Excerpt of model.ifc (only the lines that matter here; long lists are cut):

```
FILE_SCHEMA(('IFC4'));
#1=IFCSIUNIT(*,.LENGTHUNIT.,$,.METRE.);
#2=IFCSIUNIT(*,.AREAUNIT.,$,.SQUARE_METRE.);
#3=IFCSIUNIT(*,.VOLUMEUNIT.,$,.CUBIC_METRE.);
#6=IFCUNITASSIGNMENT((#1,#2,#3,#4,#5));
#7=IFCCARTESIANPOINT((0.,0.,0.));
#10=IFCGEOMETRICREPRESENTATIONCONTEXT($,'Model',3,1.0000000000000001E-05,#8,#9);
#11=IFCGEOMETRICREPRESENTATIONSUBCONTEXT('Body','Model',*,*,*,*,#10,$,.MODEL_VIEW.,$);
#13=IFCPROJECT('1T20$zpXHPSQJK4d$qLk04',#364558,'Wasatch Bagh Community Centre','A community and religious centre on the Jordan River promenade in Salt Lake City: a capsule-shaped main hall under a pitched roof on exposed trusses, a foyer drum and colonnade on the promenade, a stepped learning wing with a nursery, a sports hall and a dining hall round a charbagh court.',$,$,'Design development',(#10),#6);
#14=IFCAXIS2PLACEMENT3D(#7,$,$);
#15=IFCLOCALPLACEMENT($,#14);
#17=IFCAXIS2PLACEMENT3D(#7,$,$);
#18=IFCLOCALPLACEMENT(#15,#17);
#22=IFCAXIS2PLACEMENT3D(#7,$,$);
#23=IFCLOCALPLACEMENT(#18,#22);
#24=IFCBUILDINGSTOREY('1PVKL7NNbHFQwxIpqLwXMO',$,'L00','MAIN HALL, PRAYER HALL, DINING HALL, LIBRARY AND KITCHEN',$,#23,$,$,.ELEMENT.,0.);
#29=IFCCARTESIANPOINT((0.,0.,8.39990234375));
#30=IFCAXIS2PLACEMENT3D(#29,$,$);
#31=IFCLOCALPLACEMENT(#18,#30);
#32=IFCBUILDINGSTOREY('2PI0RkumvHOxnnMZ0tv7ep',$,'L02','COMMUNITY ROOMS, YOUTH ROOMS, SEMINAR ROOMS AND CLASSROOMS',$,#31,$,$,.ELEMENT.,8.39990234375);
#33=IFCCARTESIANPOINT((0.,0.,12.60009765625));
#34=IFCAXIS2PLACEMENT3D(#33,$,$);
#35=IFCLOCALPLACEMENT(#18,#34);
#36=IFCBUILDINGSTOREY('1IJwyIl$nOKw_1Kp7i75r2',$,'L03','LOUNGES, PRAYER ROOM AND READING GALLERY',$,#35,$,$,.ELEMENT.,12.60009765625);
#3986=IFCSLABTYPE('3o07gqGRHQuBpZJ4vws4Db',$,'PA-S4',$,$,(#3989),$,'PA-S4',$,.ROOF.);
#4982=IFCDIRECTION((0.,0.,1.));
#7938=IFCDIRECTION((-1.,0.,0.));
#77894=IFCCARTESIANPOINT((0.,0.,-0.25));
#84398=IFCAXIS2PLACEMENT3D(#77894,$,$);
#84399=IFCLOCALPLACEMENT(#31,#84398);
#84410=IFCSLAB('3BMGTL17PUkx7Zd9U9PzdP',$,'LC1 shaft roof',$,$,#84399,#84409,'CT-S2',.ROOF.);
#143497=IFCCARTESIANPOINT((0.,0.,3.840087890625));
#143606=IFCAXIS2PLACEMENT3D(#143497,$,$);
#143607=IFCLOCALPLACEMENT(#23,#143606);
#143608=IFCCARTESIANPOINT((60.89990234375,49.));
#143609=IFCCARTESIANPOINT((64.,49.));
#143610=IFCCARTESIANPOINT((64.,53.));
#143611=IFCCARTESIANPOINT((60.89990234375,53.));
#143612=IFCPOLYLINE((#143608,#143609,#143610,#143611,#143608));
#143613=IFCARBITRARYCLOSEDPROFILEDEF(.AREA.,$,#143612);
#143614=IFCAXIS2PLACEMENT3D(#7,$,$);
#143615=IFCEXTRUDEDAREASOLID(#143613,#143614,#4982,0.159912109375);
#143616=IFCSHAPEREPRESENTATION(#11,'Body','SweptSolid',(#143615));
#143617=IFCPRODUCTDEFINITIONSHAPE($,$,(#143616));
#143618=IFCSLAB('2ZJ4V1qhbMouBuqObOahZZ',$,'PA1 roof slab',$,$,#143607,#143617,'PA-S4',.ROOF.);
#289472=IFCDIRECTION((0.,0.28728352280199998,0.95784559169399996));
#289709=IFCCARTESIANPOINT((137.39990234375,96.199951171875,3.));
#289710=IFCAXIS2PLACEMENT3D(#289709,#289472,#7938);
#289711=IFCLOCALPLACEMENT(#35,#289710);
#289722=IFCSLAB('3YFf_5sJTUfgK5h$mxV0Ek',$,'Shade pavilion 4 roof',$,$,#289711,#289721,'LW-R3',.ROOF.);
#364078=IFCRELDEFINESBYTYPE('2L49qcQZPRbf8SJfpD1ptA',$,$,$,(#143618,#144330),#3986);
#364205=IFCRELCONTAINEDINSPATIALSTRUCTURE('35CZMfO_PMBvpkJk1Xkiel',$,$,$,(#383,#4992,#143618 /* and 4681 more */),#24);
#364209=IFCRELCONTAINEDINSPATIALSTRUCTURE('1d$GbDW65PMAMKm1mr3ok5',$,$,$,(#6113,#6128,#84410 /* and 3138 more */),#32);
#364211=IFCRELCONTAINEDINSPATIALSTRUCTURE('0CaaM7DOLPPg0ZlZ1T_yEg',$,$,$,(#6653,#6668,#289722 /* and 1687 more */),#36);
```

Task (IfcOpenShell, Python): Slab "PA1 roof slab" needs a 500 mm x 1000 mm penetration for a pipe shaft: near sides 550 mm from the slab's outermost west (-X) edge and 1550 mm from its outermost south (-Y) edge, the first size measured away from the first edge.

```python
import numpy as np
import ifcopenshell
import ifcopenshell.api.feature
import ifcopenshell.api.geometry
import ifcopenshell.api.root
import ifcopenshell.geom
import ifcopenshell.util.placement
import ifcopenshell.util.representation
import ifcopenshell.util.shape
import ifcopenshell.util.unit

model = ifcopenshell.open("model.ifc")
unit_scale = ifcopenshell.util.unit.calculate_unit_scale(model)
settings = ifcopenshell.geom.settings()


def volume(element):
    """Net volume in cubic metres, openings subtracted."""
    shape = ifcopenshell.geom.create_shape(settings, element)
    return ifcopenshell.util.shape.get_volume(shape.geometry)


slab = model.by_guid("2ZJ4V1qhbMouBuqObOahZZ")
before = volume(slab)

# Extent in the slab's own axes, in metres. The edges named are its -X and -Y sides.
slab_shape = ifcopenshell.geom.create_shape(settings, slab)
vertices = ifcopenshell.util.shape.get_vertices(slab_shape.geometry)
x_min, y_min, bottom = vertices.min(axis=0)
top = vertices[:, 2].max()

opening = ifcopenshell.api.root.create_entity(model, ifc_class="IfcOpeningElement", name="Pipe shaft opening", predefined_type="OPENING")
context = ifcopenshell.util.representation.get_context(model, "Model", "Body", "MODEL_VIEW")
width, depth = 0.5, 1
outline = [(0.0, 0.0), (width, 0.0), (width, depth), (0.0, depth), (0.0, 0.0)]
# Overshoot both faces by 50 mm so the cut is clean.
shape = ifcopenshell.api.geometry.add_slab_representation(
    model, context=context, depth=top - bottom + 0.1, polyline=outline
)
ifcopenshell.api.geometry.assign_representation(model, product=opening, representation=shape)

matrix = ifcopenshell.util.placement.get_local_placement(slab.ObjectPlacement)
matrix[:, 3] = matrix @ np.append(np.array([x_min + 0.55, y_min + 1.55, bottom - 0.05]) / unit_scale, 1.0)
ifcopenshell.api.geometry.edit_object_placement(model, product=opening, matrix=matrix, is_si=False)
ifcopenshell.api.feature.add_feature(model, feature=opening, element=slab)

after = volume(slab)

print(f"slab volume {before:.3f} -> {after:.3f} m3")

model.write("model_v2.ifc")
```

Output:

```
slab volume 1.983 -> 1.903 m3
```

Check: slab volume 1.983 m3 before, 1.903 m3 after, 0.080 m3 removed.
